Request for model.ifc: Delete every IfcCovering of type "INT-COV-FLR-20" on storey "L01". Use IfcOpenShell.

First a look at what the model holds.

```python
import ifcopenshell
import ifcopenshell.util.element

model = ifcopenshell.open("model.ifc")
print(model.schema)
storey = next(s for s in model.by_type("IfcBuildingStorey") if s.Name == "L01")
coverings = [e for e in ifcopenshell.util.element.get_decomposition(storey) if e.is_a("IfcCovering")]
seen = {}
for e in coverings:
    element_type = ifcopenshell.util.element.get_type(e)
    name = element_type.Name if element_type not in (None, e) else None
    seen[name] = seen.get(name, 0) + 1
for name, count in sorted(seen.items(), key=str):
    print(count, "x", name)
```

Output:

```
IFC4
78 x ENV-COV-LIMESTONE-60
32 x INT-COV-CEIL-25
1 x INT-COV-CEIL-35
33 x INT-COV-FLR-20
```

```python
import ifcopenshell
import ifcopenshell.api.root
import ifcopenshell.util.element

model = ifcopenshell.open("model.ifc")

storey = next(s for s in model.by_type("IfcBuildingStorey") if s.Name == "L01")
coverings = [e for e in ifcopenshell.util.element.get_decomposition(storey) if e.is_a("IfcCovering")]
targets = [e for e in coverings if (t := ifcopenshell.util.element.get_type(e)) not in (None, e) and t.Name == "INT-COV-FLR-20"]

for e in targets:
    ifcopenshell.api.root.remove_product(model, product=e)
print(len(targets), "removed")

model.write("model_updated.ifc")
```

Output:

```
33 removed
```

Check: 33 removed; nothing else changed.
